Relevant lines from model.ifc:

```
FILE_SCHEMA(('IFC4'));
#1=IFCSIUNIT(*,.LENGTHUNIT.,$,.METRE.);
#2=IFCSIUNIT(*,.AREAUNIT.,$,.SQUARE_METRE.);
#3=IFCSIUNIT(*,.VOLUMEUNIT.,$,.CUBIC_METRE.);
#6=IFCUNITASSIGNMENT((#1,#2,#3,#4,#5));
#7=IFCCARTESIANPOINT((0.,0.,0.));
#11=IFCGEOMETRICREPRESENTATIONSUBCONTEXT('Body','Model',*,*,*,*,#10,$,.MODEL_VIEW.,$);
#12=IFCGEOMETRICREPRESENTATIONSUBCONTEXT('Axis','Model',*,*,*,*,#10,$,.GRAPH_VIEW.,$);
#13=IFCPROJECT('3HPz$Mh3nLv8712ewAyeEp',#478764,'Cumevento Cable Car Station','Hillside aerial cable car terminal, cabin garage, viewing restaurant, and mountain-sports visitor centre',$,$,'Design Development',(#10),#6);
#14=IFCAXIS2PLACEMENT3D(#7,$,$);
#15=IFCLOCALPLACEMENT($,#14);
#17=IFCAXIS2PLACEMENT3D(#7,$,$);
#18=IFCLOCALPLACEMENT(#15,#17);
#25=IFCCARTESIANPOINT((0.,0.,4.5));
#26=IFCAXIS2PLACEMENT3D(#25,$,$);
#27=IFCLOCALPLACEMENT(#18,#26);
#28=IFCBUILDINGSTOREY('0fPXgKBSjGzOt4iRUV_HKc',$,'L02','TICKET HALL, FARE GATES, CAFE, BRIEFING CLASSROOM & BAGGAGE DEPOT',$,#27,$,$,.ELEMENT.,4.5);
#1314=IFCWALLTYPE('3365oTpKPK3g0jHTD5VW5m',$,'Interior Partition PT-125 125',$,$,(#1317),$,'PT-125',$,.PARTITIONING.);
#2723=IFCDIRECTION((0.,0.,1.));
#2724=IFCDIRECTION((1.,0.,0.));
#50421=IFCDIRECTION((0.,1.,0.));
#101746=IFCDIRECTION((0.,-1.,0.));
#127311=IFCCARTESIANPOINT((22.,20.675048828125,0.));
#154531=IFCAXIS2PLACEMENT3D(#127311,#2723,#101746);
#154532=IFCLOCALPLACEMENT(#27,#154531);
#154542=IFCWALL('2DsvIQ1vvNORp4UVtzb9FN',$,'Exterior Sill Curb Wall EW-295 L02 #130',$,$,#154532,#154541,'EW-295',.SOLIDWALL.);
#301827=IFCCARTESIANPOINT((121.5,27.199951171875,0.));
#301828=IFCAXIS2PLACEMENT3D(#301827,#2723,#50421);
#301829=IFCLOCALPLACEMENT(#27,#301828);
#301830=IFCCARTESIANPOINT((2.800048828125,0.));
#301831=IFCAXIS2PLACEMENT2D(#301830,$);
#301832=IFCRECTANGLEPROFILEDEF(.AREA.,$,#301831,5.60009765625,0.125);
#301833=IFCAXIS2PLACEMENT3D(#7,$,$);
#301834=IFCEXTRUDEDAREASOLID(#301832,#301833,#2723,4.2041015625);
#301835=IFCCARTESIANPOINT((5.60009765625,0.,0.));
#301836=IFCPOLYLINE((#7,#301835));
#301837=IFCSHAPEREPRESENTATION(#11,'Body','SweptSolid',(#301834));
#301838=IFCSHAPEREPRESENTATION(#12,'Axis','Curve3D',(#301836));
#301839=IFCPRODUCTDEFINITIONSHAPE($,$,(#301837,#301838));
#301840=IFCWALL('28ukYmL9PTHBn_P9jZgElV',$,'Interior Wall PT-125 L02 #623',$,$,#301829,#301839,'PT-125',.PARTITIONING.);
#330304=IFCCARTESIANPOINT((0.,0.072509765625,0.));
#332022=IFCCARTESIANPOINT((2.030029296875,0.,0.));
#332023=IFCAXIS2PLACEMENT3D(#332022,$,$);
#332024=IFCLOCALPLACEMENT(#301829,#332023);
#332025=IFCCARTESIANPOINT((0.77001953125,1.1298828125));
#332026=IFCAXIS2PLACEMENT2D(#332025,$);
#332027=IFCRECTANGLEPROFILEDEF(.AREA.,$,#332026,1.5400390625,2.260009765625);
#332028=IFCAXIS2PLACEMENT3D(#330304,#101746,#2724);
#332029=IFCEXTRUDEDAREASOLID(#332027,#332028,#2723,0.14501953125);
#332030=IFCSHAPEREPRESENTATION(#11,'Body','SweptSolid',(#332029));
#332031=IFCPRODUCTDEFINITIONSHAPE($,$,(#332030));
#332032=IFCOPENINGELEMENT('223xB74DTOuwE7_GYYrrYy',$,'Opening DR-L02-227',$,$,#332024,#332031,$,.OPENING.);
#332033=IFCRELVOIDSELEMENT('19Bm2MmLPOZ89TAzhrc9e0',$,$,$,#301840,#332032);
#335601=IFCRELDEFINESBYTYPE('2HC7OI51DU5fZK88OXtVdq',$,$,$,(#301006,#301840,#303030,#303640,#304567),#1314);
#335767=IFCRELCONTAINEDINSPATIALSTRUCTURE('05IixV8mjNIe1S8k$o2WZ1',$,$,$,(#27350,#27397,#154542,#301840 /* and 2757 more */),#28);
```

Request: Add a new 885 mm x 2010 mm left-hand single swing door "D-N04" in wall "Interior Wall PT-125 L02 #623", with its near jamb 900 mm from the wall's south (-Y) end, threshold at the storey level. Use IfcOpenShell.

```python
import numpy as np
import ifcopenshell
import ifcopenshell.api.feature
import ifcopenshell.api.geometry
import ifcopenshell.api.root
import ifcopenshell.api.spatial
import ifcopenshell.geom
import ifcopenshell.util.element
import ifcopenshell.util.placement
import ifcopenshell.util.representation
import ifcopenshell.util.shape
import ifcopenshell.util.unit

model = ifcopenshell.open("model.ifc")
unit_scale = ifcopenshell.util.unit.calculate_unit_scale(model)
settings = ifcopenshell.geom.settings()


def volume(element):
    """Net volume in cubic metres, openings subtracted."""
    shape = ifcopenshell.geom.create_shape(settings, element)
    return ifcopenshell.util.shape.get_volume(shape.geometry)


wall = model.by_guid("28ukYmL9PTHBn_P9jZgElV")
storey = ifcopenshell.util.element.get_container(wall, ifc_class="IfcBuildingStorey")
context = ifcopenshell.util.representation.get_context(model, "Model", "Body", "MODEL_VIEW")
before = volume(wall)

width, height, from_end, sill = 0.885, 2.01, 0.9, 0.0  # metres

# The wall runs along its own X axis, and the end named is its -X end.
wall_shape = ifcopenshell.geom.create_shape(settings, wall)
x, y, z = ifcopenshell.util.shape.get_vertices(wall_shape.geometry).T
start = x.min() + from_end
face, thickness = float(y.min()), float(y.max() - y.min())
wall_matrix = ifcopenshell.util.placement.get_local_placement(wall.ObjectPlacement)
level = ifcopenshell.util.placement.get_local_placement(storey.ObjectPlacement)[2, 3]


def in_wall(x, y):
    """Placement at x, y metres in the wall's axes, at sill height."""
    matrix = wall_matrix.copy()
    matrix[:, 3] = wall_matrix @ np.array([x / unit_scale, y / unit_scale, 0.0, 1.0])
    matrix[2, 3] = level + sill / unit_scale
    return matrix


# Opening: a box that overshoots both wall faces by 50 mm.
opening = ifcopenshell.api.root.create_entity(model, ifc_class="IfcOpeningElement", predefined_type="OPENING")
box = ifcopenshell.api.geometry.add_wall_representation(
    model, context=context, length=width, height=height, thickness=thickness + 0.1
)
ifcopenshell.api.geometry.assign_representation(model, product=opening, representation=box)
ifcopenshell.api.geometry.edit_object_placement(model, product=opening, matrix=in_wall(start, face - 0.05), is_si=False)
ifcopenshell.api.feature.add_feature(model, feature=opening, element=wall)

door = ifcopenshell.api.root.create_entity(model, ifc_class="IfcDoor", name="D-N04", predefined_type="DOOR")
door.OverallWidth, door.OverallHeight = width / unit_scale, height / unit_scale
door.OperationType = "SINGLE_SWING_LEFT"
body = ifcopenshell.api.geometry.add_door_representation(
    model,
    context=context,
    overall_width=door.OverallWidth,
    overall_height=door.OverallHeight,
    operation_type="SINGLE_SWING_LEFT",
    lining_properties={"LiningDepth": thickness / unit_scale, "ThresholdDepth": thickness / unit_scale},
)
ifcopenshell.api.geometry.assign_representation(model, product=door, representation=body)
ifcopenshell.api.spatial.assign_container(model, products=[door], relating_structure=storey)
ifcopenshell.api.feature.add_filling(model, opening=opening, element=door)

# The lining spans the wall, so the door starts at the wall face.
ifcopenshell.api.geometry.edit_object_placement(model, product=door, matrix=in_wall(start, face), is_si=False)

after = volume(wall)

print(f"wall volume {before:.3f} -> {after:.3f} m3")

model.write("model_edited.ifc")
```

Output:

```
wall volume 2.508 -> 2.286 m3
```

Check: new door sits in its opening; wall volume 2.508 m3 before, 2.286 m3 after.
